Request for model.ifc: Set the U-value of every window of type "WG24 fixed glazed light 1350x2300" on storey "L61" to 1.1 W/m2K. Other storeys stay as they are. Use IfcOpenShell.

First a look at what the model holds.

```python
import ifcopenshell
import ifcopenshell.util.element

model = ifcopenshell.open("model.ifc")
print(model.schema)
storey = next(s for s in model.by_type("IfcBuildingStorey") if s.Name == "L61")
windows = [e for e in ifcopenshell.util.element.get_decomposition(storey) if e.is_a("IfcWindow")]
seen = {}
for e in windows:
    element_type = ifcopenshell.util.element.get_type(e)
    key = (element_type.Name if element_type != e and element_type else None, ifcopenshell.util.element.get_pset(e, "Pset_WindowCommon", "ThermalTransmittance"))
    seen[key] = seen.get(key, 0) + 1
for (name, value), count in sorted(seen.items(), key=str):
    print(count, "x", name, "|", value)
```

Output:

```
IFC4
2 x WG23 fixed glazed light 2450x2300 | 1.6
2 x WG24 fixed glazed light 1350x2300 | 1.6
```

```python
import ifcopenshell
import ifcopenshell.api.pset
import ifcopenshell.util.element

model = ifcopenshell.open("model.ifc")

storey = next(s for s in model.by_type("IfcBuildingStorey") if s.Name == "L61")
windows = [e for e in ifcopenshell.util.element.get_decomposition(storey) if e.is_a("IfcWindow")]

count = 0
for e in windows:
    element_type = ifcopenshell.util.element.get_type(e)
    if element_type in (None, e) or element_type.Name != "WG24 fixed glazed light 1350x2300":
        continue
    # add_pset returns the element's existing set when there is one.
    pset = ifcopenshell.api.pset.add_pset(model, product=e, name="Pset_WindowCommon")
    ifcopenshell.api.pset.edit_pset(model, pset=pset, properties={"ThermalTransmittance": 1.1})
    count += 1

print(count, "windows updated")

model.write("model_edited.ifc")
```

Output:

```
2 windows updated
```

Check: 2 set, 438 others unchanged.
